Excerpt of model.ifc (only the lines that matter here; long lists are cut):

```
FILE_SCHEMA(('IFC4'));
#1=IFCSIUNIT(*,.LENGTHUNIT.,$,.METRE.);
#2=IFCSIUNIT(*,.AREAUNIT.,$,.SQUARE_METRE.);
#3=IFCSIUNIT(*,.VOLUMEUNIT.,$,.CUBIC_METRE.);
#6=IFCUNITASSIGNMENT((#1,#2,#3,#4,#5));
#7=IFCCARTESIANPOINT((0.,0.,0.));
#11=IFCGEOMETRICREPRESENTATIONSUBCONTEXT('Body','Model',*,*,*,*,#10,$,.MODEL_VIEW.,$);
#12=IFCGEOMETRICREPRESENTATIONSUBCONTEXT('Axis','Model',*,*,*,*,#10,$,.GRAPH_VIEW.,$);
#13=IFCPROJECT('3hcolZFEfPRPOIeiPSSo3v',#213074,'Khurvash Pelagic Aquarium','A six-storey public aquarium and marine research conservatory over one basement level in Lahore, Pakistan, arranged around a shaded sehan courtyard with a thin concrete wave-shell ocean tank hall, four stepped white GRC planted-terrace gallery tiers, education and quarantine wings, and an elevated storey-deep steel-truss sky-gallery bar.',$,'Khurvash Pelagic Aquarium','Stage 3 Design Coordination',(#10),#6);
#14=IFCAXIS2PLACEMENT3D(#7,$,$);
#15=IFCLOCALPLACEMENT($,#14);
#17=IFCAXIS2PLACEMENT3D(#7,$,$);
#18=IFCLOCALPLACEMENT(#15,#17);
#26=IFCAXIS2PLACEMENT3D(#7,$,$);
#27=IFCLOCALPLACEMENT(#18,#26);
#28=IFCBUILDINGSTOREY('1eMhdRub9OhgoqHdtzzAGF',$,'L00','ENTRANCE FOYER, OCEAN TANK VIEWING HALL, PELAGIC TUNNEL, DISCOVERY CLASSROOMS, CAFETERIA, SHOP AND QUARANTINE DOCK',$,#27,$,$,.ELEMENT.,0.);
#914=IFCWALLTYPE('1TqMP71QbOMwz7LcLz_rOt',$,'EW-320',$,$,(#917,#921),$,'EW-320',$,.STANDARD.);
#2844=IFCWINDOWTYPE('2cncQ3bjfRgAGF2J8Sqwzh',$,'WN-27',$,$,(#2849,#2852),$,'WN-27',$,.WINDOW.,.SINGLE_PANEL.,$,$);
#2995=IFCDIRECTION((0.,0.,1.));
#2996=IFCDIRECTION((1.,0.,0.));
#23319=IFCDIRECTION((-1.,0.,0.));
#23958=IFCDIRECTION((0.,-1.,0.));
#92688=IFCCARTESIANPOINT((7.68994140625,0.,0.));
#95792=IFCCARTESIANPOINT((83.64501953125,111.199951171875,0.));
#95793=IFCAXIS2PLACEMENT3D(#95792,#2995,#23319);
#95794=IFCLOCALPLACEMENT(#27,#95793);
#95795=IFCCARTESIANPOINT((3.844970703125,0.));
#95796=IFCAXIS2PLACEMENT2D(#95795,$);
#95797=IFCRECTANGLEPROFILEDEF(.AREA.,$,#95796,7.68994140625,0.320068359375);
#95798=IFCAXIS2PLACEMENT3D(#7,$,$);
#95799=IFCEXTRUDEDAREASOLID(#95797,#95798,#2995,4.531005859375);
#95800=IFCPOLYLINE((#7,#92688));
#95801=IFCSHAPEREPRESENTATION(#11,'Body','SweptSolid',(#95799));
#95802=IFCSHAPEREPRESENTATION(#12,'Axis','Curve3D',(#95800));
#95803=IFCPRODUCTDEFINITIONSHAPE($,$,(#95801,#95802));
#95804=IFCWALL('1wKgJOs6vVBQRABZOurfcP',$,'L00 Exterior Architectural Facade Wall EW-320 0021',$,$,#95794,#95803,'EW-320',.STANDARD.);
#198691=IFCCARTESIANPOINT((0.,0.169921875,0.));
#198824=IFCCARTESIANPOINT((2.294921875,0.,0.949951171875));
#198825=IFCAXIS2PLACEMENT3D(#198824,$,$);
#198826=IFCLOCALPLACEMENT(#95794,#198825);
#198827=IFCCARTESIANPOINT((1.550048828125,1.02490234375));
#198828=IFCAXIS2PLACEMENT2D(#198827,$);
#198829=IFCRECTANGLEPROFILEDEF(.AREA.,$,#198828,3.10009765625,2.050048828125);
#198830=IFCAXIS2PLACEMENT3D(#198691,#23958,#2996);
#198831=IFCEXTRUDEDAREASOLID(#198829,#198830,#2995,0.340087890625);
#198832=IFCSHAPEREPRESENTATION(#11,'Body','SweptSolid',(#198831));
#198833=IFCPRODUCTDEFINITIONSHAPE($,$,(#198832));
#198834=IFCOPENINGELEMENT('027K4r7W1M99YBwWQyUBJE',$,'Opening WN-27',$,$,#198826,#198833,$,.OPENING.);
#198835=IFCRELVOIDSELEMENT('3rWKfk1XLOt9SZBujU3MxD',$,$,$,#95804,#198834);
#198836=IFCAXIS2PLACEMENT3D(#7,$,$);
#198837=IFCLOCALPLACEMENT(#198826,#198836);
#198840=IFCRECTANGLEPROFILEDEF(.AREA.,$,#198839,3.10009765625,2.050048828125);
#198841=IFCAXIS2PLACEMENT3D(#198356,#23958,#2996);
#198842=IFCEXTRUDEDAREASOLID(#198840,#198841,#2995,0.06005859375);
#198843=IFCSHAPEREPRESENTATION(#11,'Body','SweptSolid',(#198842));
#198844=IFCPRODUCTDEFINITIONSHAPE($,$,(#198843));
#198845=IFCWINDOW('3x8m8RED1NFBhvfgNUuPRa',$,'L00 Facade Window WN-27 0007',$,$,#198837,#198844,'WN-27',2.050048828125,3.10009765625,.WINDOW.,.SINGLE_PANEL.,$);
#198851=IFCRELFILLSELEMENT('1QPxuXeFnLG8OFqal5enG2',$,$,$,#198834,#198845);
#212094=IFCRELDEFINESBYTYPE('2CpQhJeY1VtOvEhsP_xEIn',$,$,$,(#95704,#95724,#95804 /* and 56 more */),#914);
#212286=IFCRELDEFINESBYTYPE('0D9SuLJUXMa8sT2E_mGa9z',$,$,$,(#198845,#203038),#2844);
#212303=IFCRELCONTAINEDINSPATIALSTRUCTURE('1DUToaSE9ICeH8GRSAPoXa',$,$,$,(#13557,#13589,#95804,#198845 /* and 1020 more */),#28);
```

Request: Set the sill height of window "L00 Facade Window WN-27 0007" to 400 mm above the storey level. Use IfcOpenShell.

```python
import numpy as np
import ifcopenshell
import ifcopenshell.api.geometry
import ifcopenshell.geom
import ifcopenshell.util.element
import ifcopenshell.util.placement
import ifcopenshell.util.shape
import ifcopenshell.util.unit

model = ifcopenshell.open("model.ifc")
unit_scale = ifcopenshell.util.unit.calculate_unit_scale(model)

window = model.by_id(198845)
opening = window.FillsVoids[0].RelatingOpeningElement
storey = ifcopenshell.util.element.get_container(window, ifc_class="IfcBuildingStorey")
level = ifcopenshell.util.placement.get_local_placement(storey.ObjectPlacement)[2, 3]

# The opening's origin need not be at the sill, so measure its lowest point.
shape = ifcopenshell.geom.create_shape(ifcopenshell.geom.settings(), opening)
bottom = ifcopenshell.util.shape.get_shape_bottom_elevation(shape, shape.geometry) / unit_scale
dz = level + 0.4 / unit_scale - bottom

shift = np.array([0.0, 0.0, dz])
# The window is placed relative to its opening, so it follows when the opening moves.
matrix = ifcopenshell.util.placement.get_local_placement(opening.ObjectPlacement)
matrix[:3, 3] += shift
ifcopenshell.api.geometry.edit_object_placement(
    model, product=opening, matrix=matrix, is_si=False, should_transform_children=True
)

print(f"moved by {dz * unit_scale:+.3f} m")

model.write("model_updated.ifc")
```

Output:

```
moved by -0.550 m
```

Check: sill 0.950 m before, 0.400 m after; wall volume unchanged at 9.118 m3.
